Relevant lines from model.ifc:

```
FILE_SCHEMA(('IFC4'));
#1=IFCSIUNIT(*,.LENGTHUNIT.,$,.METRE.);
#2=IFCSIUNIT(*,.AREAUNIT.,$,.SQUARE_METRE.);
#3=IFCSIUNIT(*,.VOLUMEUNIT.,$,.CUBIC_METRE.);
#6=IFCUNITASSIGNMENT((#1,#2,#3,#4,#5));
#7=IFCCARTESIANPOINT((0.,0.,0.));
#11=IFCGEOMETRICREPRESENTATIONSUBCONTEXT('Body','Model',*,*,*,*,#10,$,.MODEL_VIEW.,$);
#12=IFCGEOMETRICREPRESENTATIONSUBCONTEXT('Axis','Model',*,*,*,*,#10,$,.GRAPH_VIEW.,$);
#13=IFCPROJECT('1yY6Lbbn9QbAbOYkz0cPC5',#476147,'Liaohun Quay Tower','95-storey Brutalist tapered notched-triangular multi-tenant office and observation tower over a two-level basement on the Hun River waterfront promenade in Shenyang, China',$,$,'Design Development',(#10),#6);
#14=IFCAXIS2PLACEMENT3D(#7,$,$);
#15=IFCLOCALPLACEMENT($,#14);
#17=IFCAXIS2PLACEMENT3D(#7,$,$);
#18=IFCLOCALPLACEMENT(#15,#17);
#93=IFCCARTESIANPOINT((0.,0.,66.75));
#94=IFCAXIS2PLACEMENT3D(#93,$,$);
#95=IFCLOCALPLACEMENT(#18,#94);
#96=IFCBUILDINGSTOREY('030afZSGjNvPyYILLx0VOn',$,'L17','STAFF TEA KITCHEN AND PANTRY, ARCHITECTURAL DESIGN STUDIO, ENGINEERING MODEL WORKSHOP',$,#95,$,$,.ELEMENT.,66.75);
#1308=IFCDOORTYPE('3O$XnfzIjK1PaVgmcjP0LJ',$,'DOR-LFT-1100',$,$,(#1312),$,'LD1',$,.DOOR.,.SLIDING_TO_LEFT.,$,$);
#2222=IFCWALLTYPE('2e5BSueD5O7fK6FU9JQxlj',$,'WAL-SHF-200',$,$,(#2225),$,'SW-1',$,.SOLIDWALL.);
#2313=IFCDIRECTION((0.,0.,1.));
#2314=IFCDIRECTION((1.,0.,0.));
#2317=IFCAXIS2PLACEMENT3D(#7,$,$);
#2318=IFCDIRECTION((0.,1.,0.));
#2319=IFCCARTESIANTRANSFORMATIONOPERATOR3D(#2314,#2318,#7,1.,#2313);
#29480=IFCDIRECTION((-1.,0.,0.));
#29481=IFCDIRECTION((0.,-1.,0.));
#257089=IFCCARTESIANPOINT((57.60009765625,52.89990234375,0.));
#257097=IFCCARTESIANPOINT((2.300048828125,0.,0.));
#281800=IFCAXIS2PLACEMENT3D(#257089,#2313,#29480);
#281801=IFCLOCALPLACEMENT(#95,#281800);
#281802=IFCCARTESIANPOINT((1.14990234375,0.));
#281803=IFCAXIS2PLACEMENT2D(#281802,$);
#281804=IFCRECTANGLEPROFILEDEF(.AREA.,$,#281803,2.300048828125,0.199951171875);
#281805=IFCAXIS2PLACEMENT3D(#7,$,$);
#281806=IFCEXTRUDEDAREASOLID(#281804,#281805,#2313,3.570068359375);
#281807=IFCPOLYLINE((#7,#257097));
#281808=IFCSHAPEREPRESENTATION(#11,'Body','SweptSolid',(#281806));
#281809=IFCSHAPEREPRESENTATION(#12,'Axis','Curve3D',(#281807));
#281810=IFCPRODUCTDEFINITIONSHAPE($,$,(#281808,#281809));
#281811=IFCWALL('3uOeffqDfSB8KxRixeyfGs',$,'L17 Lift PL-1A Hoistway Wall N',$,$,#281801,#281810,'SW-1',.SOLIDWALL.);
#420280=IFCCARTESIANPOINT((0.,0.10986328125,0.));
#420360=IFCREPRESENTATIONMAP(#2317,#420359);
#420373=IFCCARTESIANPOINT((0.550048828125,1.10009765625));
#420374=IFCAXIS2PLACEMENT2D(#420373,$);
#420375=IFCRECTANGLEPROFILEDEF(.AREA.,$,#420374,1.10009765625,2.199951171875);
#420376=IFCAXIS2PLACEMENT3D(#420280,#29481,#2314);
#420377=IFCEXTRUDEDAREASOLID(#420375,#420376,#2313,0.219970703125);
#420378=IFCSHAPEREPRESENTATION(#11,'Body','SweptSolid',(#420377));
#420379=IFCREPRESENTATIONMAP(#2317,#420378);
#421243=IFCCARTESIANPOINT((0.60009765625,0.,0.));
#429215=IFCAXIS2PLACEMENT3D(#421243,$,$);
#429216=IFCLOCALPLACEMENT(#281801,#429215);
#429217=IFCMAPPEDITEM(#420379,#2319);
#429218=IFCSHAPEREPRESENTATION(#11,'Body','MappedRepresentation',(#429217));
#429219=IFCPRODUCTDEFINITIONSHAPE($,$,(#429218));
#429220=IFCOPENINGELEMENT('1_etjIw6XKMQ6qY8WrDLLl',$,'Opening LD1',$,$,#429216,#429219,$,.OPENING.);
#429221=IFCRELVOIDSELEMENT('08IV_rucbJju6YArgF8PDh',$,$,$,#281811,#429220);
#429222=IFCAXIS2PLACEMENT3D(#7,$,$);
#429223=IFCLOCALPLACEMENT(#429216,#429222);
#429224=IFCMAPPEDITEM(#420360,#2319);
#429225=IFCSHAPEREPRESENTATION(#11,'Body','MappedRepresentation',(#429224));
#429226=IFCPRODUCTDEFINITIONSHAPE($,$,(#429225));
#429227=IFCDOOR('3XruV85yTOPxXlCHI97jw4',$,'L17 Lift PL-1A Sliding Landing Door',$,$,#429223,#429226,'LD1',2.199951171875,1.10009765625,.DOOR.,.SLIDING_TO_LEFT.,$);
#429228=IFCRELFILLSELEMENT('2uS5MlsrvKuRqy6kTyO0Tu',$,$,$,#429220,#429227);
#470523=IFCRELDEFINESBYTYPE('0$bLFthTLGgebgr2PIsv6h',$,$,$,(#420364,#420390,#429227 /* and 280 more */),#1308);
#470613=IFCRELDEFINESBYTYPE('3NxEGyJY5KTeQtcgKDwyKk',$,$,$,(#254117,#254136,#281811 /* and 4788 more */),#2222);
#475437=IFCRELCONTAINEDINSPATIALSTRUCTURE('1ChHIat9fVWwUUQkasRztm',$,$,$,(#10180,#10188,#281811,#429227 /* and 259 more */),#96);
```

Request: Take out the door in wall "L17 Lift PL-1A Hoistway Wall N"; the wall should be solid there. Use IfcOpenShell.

```python
import ifcopenshell
import ifcopenshell.api.feature
import ifcopenshell.api.root
import ifcopenshell.geom
import ifcopenshell.util.shape

model = ifcopenshell.open("model.ifc")
settings = ifcopenshell.geom.settings()


def volume(element):
    """Net volume in cubic metres, openings subtracted."""
    shape = ifcopenshell.geom.create_shape(settings, element)
    return ifcopenshell.util.shape.get_volume(shape.geometry)


door = model.by_id(429227)
opening = door.FillsVoids[0].RelatingOpeningElement
wall = opening.VoidsElements[0].RelatingBuildingElement
before = volume(wall)

ifcopenshell.api.root.remove_product(model, product=door)
ifcopenshell.api.feature.remove_feature(model, feature=opening)

after = volume(wall)

print(f"wall volume {before:.3f} -> {after:.3f} m3")

model.write("model-out.ifc")
```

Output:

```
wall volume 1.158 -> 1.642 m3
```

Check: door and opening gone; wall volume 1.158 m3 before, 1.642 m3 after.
